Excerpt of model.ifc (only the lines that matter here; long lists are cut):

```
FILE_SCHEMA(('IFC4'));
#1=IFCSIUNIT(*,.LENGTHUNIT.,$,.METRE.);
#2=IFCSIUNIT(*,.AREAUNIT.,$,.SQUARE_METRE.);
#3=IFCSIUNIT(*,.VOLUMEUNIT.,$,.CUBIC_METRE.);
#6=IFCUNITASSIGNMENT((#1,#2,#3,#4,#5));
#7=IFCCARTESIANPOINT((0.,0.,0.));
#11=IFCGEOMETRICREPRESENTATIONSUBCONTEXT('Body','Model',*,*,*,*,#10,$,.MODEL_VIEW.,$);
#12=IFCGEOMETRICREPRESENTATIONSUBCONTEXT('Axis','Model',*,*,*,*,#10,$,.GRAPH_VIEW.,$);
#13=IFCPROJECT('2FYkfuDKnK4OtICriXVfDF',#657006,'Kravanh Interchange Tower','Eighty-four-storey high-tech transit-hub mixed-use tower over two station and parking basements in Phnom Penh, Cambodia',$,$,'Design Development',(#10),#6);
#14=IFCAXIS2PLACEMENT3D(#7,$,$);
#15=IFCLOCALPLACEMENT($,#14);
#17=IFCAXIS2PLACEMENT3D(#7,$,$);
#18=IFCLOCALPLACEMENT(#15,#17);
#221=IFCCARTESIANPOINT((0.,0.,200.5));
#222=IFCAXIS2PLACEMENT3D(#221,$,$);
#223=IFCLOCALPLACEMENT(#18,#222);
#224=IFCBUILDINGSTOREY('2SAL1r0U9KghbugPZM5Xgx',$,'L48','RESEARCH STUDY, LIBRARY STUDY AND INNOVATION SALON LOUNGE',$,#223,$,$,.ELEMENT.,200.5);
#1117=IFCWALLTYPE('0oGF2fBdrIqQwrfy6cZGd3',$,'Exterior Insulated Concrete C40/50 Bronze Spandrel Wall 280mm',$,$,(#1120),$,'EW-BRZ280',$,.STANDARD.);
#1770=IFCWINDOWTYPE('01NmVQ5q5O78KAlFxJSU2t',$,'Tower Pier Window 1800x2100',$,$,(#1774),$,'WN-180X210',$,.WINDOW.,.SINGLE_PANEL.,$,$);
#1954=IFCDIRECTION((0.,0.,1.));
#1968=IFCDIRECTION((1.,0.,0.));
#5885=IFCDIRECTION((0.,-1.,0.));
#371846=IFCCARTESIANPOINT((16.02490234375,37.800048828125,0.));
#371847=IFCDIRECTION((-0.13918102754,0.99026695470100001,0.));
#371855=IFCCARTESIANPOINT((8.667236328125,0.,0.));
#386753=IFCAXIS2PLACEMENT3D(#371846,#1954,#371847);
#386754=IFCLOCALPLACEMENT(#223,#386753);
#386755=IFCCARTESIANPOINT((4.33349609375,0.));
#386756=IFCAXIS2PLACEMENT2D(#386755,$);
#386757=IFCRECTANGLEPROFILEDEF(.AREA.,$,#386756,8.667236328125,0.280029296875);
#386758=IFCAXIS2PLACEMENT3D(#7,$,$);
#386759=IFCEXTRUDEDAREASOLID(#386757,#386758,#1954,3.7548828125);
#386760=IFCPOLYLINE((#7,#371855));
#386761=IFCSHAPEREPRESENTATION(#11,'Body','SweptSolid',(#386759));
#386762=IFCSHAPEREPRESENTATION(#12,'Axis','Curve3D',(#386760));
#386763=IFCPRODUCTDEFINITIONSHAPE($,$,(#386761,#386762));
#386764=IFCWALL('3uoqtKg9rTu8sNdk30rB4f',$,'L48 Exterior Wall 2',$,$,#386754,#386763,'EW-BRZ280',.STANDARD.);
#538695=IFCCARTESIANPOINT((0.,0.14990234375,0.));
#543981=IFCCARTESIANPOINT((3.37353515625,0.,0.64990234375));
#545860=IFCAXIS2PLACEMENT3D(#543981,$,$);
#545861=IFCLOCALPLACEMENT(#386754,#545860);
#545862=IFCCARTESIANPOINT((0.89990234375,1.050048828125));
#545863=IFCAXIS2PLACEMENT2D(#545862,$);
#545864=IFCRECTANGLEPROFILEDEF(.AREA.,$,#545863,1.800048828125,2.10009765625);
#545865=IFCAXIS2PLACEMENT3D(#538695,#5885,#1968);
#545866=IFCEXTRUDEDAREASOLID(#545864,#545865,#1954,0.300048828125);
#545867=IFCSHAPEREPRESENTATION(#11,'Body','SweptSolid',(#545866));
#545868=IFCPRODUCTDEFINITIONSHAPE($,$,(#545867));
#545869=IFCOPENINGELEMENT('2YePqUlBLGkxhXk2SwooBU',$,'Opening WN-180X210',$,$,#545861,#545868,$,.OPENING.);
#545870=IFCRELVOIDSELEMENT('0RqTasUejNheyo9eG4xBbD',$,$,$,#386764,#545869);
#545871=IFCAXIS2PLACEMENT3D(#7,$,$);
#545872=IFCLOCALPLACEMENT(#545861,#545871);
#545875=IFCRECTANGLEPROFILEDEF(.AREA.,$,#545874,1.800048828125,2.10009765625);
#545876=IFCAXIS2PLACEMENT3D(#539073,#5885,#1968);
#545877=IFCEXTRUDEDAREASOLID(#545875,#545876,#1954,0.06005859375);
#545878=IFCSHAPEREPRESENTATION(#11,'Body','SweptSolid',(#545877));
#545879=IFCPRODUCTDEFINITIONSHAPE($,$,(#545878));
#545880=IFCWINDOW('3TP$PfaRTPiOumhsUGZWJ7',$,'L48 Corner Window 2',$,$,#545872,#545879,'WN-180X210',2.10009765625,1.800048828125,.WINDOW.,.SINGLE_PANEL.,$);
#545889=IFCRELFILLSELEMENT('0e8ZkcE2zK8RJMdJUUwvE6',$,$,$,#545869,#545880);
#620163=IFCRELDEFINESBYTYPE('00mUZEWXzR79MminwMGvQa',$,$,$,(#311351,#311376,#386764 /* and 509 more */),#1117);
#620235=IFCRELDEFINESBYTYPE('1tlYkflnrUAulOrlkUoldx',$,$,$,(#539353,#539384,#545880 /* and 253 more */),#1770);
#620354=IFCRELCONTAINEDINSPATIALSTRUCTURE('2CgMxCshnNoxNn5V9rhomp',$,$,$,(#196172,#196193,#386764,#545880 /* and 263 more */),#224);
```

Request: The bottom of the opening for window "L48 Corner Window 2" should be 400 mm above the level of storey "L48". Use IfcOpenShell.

```python
import numpy as np
import ifcopenshell
import ifcopenshell.api.geometry
import ifcopenshell.geom
import ifcopenshell.util.element
import ifcopenshell.util.placement
import ifcopenshell.util.shape
import ifcopenshell.util.unit

model = ifcopenshell.open("model.ifc")
unit_scale = ifcopenshell.util.unit.calculate_unit_scale(model)

window = model.by_guid("3TP$PfaRTPiOumhsUGZWJ7")
opening = window.FillsVoids[0].RelatingOpeningElement
storey = ifcopenshell.util.element.get_container(window, ifc_class="IfcBuildingStorey")
level = ifcopenshell.util.placement.get_local_placement(storey.ObjectPlacement)[2, 3]

# The opening's origin need not be at the sill, so measure its lowest point.
shape = ifcopenshell.geom.create_shape(ifcopenshell.geom.settings(), opening)
bottom = ifcopenshell.util.shape.get_shape_bottom_elevation(shape, shape.geometry) / unit_scale
dz = level + 0.4 / unit_scale - bottom

shift = np.array([0.0, 0.0, dz])
# The window is placed relative to its opening, so it follows when the opening moves.
matrix = ifcopenshell.util.placement.get_local_placement(opening.ObjectPlacement)
matrix[:3, 3] += shift
ifcopenshell.api.geometry.edit_object_placement(
    model, product=opening, matrix=matrix, is_si=False, should_transform_children=True
)

print(f"moved by {dz * unit_scale:+.3f} m")

model.write("model-out.ifc")
```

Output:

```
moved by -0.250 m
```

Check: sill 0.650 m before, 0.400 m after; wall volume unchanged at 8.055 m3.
